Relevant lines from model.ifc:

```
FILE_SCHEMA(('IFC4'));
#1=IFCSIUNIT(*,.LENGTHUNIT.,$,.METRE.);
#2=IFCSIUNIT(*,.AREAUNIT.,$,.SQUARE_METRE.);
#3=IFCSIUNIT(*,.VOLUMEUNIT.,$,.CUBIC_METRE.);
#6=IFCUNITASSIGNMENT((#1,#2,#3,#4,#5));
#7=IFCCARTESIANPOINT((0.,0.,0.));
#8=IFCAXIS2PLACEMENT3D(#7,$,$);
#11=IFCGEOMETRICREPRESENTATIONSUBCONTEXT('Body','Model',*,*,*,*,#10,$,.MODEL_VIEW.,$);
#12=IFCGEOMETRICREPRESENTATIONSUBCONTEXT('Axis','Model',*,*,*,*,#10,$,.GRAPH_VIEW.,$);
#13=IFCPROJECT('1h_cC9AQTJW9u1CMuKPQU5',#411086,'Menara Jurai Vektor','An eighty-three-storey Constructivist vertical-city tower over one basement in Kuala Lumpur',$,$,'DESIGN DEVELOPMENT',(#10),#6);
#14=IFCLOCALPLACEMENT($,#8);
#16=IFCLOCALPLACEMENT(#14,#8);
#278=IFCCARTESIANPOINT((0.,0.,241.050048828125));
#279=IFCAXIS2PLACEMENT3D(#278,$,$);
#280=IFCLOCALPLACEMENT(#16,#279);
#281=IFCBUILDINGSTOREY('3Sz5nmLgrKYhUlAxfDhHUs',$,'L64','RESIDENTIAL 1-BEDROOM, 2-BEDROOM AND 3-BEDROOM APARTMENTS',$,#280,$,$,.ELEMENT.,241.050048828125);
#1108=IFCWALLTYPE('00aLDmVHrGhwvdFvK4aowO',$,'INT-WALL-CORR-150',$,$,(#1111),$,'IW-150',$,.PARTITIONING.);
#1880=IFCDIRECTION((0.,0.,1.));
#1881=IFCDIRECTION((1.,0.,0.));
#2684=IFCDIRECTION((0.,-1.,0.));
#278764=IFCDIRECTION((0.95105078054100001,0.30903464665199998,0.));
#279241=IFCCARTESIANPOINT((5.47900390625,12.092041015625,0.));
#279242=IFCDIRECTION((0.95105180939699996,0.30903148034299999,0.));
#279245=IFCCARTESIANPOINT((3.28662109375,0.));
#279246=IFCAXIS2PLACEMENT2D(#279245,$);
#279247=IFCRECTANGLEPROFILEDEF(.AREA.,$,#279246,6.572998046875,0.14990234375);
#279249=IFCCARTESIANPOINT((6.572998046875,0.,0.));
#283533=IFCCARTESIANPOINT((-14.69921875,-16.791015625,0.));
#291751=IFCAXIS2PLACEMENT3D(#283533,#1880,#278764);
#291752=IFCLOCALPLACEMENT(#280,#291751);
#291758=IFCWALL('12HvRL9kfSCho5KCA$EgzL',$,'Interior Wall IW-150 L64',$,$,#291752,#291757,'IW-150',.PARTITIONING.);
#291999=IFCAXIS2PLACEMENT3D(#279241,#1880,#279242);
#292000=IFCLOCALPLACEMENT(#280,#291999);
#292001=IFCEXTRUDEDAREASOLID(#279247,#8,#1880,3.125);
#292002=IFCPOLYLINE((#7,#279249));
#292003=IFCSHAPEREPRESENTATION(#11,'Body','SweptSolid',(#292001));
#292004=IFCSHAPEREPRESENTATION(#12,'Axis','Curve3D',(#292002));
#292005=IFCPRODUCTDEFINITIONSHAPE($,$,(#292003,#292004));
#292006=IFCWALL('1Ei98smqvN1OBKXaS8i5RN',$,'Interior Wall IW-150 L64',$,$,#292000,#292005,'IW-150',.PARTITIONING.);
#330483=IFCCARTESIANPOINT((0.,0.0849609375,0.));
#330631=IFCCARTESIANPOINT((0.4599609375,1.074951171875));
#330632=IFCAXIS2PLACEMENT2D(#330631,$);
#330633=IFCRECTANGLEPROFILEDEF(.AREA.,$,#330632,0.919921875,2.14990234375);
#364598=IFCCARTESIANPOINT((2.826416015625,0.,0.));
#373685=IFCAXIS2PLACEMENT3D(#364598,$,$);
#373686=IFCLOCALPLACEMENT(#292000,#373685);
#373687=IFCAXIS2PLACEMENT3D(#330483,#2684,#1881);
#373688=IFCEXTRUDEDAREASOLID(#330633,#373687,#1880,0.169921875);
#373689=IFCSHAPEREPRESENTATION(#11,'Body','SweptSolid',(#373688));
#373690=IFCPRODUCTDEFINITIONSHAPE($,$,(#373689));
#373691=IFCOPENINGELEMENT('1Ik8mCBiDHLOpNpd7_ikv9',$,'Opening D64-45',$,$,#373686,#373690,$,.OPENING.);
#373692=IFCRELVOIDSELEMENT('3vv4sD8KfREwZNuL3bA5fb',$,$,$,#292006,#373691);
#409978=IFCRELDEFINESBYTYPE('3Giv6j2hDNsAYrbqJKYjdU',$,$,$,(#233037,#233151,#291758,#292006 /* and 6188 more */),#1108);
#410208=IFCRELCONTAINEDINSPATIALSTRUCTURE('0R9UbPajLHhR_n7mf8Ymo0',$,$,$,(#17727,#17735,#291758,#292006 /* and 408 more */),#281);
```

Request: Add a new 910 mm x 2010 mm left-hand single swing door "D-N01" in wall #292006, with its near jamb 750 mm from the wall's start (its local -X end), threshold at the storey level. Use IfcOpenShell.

```python
import numpy as np
import ifcopenshell
import ifcopenshell.api.feature
import ifcopenshell.api.geometry
import ifcopenshell.api.root
import ifcopenshell.api.spatial
import ifcopenshell.geom
import ifcopenshell.util.element
import ifcopenshell.util.placement
import ifcopenshell.util.representation
import ifcopenshell.util.shape
import ifcopenshell.util.unit

model = ifcopenshell.open("model.ifc")
unit_scale = ifcopenshell.util.unit.calculate_unit_scale(model)
settings = ifcopenshell.geom.settings()


def volume(element):
    """Net volume in cubic metres, openings subtracted."""
    shape = ifcopenshell.geom.create_shape(settings, element)
    return ifcopenshell.util.shape.get_volume(shape.geometry)


wall = model.by_guid("1Ei98smqvN1OBKXaS8i5RN")
storey = ifcopenshell.util.element.get_container(wall, ifc_class="IfcBuildingStorey")
context = ifcopenshell.util.representation.get_context(model, "Model", "Body", "MODEL_VIEW")
before = volume(wall)

width, height, from_end, sill = 0.91, 2.01, 0.75, 0.0  # metres

# The wall runs along its own X axis, and the end named is its -X end.
wall_shape = ifcopenshell.geom.create_shape(settings, wall)
x, y, z = ifcopenshell.util.shape.get_vertices(wall_shape.geometry).T
start = x.min() + from_end
face, thickness = float(y.min()), float(y.max() - y.min())
wall_matrix = ifcopenshell.util.placement.get_local_placement(wall.ObjectPlacement)
level = ifcopenshell.util.placement.get_local_placement(storey.ObjectPlacement)[2, 3]


def in_wall(x, y):
    """Placement at x, y metres in the wall's axes, at sill height."""
    matrix = wall_matrix.copy()
    matrix[:, 3] = wall_matrix @ np.array([x / unit_scale, y / unit_scale, 0.0, 1.0])
    matrix[2, 3] = level + sill / unit_scale
    return matrix


# Opening: a box that overshoots both wall faces by 50 mm.
opening = ifcopenshell.api.root.create_entity(model, ifc_class="IfcOpeningElement", predefined_type="OPENING")
box = ifcopenshell.api.geometry.add_wall_representation(
    model, context=context, length=width, height=height, thickness=thickness + 0.1
)
ifcopenshell.api.geometry.assign_representation(model, product=opening, representation=box)
ifcopenshell.api.geometry.edit_object_placement(model, product=opening, matrix=in_wall(start, face - 0.05), is_si=False)
ifcopenshell.api.feature.add_feature(model, feature=opening, element=wall)

door = ifcopenshell.api.root.create_entity(model, ifc_class="IfcDoor", name="D-N01", predefined_type="DOOR")
door.OverallWidth, door.OverallHeight = width / unit_scale, height / unit_scale
door.OperationType = "SINGLE_SWING_LEFT"
body = ifcopenshell.api.geometry.add_door_representation(
    model,
    context=context,
    overall_width=door.OverallWidth,
    overall_height=door.OverallHeight,
    operation_type="SINGLE_SWING_LEFT",
    lining_properties={"LiningDepth": thickness / unit_scale, "ThresholdDepth": thickness / unit_scale},
)
ifcopenshell.api.geometry.assign_representation(model, product=door, representation=body)
ifcopenshell.api.spatial.assign_container(model, products=[door], relating_structure=storey)
ifcopenshell.api.feature.add_filling(model, opening=opening, element=door)

# The lining spans the wall, so the door starts at the wall face.
ifcopenshell.api.geometry.edit_object_placement(model, product=door, matrix=in_wall(start, face), is_si=False)

after = volume(wall)

print(f"wall volume {before:.3f} -> {after:.3f} m3")

model.write("model_edited.ifc")
```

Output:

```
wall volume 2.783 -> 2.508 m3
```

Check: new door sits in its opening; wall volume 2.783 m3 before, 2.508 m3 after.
